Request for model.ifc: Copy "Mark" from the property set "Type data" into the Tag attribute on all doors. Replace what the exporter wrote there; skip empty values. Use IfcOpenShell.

First a look at what the model holds.

```python
import ifcopenshell
import ifcopenshell.util.element

model = ifcopenshell.open("model.ifc")
print(model.schema)
doors = model.by_type("IfcDoor")
print(len(doors), "doors")
for e in doors[:8]:
    source = ifcopenshell.util.element.get_pset(e, "Type data", "Mark")
    target = e.Tag
    print(e.id(), repr(source), repr(target), sep=" | ")
```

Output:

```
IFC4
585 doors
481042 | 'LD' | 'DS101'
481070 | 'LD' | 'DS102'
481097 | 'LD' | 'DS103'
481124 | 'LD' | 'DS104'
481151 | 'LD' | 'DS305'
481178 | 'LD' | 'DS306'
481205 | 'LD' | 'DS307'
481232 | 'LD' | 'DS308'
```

```python
import ifcopenshell
import ifcopenshell.util.element

model = ifcopenshell.open("model.ifc")

count = 0
for e in model.by_type("IfcDoor"):
    value = ifcopenshell.util.element.get_pset(e, "Type data", "Mark")
    current = e.Tag
    if not value or not value.strip() or current == value:
        continue
    e.Tag = value
    count += 1

print(count, "doors updated")

model.write("model_updated.ifc")
```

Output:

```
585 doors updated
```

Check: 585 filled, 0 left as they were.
